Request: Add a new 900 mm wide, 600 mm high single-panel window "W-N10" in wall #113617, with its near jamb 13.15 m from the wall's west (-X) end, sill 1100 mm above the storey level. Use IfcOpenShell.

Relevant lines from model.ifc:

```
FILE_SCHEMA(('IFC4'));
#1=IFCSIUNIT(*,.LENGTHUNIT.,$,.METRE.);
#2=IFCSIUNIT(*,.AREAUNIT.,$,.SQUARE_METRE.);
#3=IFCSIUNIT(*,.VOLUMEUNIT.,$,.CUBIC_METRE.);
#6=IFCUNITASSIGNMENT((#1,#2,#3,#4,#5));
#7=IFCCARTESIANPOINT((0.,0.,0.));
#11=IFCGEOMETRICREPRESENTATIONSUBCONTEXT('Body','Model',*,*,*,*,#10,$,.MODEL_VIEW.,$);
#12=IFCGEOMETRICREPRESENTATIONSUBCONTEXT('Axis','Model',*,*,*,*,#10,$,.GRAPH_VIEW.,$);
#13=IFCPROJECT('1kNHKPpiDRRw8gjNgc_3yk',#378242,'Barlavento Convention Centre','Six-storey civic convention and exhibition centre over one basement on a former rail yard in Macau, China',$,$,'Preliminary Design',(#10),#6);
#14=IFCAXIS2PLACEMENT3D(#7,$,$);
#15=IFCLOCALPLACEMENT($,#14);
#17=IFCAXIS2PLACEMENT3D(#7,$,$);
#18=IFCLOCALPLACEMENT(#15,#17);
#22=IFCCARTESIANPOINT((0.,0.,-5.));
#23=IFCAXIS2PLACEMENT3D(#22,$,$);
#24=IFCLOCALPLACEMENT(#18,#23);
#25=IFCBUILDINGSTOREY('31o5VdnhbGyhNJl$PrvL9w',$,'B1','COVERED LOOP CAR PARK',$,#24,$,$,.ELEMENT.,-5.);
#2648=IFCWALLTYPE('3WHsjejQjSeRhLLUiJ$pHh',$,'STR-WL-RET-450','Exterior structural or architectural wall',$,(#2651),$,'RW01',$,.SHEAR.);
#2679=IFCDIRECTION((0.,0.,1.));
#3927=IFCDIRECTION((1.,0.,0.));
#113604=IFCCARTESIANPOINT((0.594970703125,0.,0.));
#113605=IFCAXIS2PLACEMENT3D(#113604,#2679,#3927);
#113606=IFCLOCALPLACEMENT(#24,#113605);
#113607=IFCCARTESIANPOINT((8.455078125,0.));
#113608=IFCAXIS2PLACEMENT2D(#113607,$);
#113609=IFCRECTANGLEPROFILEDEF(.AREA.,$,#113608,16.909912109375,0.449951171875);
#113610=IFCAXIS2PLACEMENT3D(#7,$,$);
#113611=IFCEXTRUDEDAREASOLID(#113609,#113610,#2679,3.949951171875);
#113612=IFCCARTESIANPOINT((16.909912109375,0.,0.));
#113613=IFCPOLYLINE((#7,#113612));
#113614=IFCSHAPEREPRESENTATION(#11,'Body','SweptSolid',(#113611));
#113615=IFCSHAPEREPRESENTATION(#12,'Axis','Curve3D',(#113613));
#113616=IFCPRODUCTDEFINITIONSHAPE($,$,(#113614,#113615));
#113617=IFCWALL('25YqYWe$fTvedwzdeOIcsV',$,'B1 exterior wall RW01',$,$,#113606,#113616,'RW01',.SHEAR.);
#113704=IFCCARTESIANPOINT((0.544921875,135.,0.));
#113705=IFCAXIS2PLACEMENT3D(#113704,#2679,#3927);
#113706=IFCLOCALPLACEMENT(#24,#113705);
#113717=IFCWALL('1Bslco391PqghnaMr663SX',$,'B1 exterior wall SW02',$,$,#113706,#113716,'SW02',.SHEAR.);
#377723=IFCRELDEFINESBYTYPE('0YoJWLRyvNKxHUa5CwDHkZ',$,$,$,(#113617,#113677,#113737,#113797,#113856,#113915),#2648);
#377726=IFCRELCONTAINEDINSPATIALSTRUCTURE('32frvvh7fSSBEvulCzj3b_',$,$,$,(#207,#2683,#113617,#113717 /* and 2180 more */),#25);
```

```python
import numpy as np
import ifcopenshell
import ifcopenshell.api.feature
import ifcopenshell.api.geometry
import ifcopenshell.api.root
import ifcopenshell.api.spatial
import ifcopenshell.geom
import ifcopenshell.util.element
import ifcopenshell.util.placement
import ifcopenshell.util.representation
import ifcopenshell.util.shape
import ifcopenshell.util.unit

model = ifcopenshell.open("model.ifc")
unit_scale = ifcopenshell.util.unit.calculate_unit_scale(model)
settings = ifcopenshell.geom.settings()


def volume(element):
    """Net volume in cubic metres, openings subtracted."""
    shape = ifcopenshell.geom.create_shape(settings, element)
    return ifcopenshell.util.shape.get_volume(shape.geometry)


wall = model.by_id(113617)
storey = ifcopenshell.util.element.get_container(wall, ifc_class="IfcBuildingStorey")
context = ifcopenshell.util.representation.get_context(model, "Model", "Body", "MODEL_VIEW")
before = volume(wall)

width, height, from_end, sill = 0.9, 0.6, 13.15, 1.1  # metres

# The wall runs along its own X axis, and the end named is its -X end.
wall_shape = ifcopenshell.geom.create_shape(settings, wall)
x, y, z = ifcopenshell.util.shape.get_vertices(wall_shape.geometry).T
start = x.min() + from_end
face, thickness = float(y.min()), float(y.max() - y.min())
wall_matrix = ifcopenshell.util.placement.get_local_placement(wall.ObjectPlacement)
level = ifcopenshell.util.placement.get_local_placement(storey.ObjectPlacement)[2, 3]


def in_wall(x, y):
    """Placement at x, y metres in the wall's axes, at sill height."""
    matrix = wall_matrix.copy()
    matrix[:, 3] = wall_matrix @ np.array([x / unit_scale, y / unit_scale, 0.0, 1.0])
    matrix[2, 3] = level + sill / unit_scale
    return matrix


# Opening: a box that overshoots both wall faces by 50 mm.
opening = ifcopenshell.api.root.create_entity(model, ifc_class="IfcOpeningElement", predefined_type="OPENING")
box = ifcopenshell.api.geometry.add_wall_representation(
    model, context=context, length=width, height=height, thickness=thickness + 0.1
)
ifcopenshell.api.geometry.assign_representation(model, product=opening, representation=box)
ifcopenshell.api.geometry.edit_object_placement(model, product=opening, matrix=in_wall(start, face - 0.05), is_si=False)
ifcopenshell.api.feature.add_feature(model, feature=opening, element=wall)

window = ifcopenshell.api.root.create_entity(model, ifc_class="IfcWindow", name="W-N10", predefined_type="WINDOW")
window.OverallWidth, window.OverallHeight = width / unit_scale, height / unit_scale
window.PartitioningType = "SINGLE_PANEL"
body = ifcopenshell.api.geometry.add_window_representation(
    model,
    context=context,
    overall_width=window.OverallWidth,
    overall_height=window.OverallHeight,
    partition_type="SINGLE_PANEL",
)
ifcopenshell.api.geometry.assign_representation(model, product=window, representation=body)
ifcopenshell.api.spatial.assign_container(model, products=[window], relating_structure=storey)
ifcopenshell.api.feature.add_filling(model, opening=opening, element=window)

# Centre the window in the wall's thickness.
ifcopenshell.api.geometry.edit_object_placement(model, product=window, matrix=in_wall(start, face), is_si=False)
window_shape = ifcopenshell.geom.create_shape(settings, window)
depth = ifcopenshell.util.shape.get_vertices(window_shape.geometry)[:, 1]
offset = face + thickness / 2 - (depth.min() + depth.max()) / 2
ifcopenshell.api.geometry.edit_object_placement(model, product=window, matrix=in_wall(start, offset), is_si=False)

after = volume(wall)

print(f"wall volume {before:.3f} -> {after:.3f} m3")

model.write("model_edited.ifc")
```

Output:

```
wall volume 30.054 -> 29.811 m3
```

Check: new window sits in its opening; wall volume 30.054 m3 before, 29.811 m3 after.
